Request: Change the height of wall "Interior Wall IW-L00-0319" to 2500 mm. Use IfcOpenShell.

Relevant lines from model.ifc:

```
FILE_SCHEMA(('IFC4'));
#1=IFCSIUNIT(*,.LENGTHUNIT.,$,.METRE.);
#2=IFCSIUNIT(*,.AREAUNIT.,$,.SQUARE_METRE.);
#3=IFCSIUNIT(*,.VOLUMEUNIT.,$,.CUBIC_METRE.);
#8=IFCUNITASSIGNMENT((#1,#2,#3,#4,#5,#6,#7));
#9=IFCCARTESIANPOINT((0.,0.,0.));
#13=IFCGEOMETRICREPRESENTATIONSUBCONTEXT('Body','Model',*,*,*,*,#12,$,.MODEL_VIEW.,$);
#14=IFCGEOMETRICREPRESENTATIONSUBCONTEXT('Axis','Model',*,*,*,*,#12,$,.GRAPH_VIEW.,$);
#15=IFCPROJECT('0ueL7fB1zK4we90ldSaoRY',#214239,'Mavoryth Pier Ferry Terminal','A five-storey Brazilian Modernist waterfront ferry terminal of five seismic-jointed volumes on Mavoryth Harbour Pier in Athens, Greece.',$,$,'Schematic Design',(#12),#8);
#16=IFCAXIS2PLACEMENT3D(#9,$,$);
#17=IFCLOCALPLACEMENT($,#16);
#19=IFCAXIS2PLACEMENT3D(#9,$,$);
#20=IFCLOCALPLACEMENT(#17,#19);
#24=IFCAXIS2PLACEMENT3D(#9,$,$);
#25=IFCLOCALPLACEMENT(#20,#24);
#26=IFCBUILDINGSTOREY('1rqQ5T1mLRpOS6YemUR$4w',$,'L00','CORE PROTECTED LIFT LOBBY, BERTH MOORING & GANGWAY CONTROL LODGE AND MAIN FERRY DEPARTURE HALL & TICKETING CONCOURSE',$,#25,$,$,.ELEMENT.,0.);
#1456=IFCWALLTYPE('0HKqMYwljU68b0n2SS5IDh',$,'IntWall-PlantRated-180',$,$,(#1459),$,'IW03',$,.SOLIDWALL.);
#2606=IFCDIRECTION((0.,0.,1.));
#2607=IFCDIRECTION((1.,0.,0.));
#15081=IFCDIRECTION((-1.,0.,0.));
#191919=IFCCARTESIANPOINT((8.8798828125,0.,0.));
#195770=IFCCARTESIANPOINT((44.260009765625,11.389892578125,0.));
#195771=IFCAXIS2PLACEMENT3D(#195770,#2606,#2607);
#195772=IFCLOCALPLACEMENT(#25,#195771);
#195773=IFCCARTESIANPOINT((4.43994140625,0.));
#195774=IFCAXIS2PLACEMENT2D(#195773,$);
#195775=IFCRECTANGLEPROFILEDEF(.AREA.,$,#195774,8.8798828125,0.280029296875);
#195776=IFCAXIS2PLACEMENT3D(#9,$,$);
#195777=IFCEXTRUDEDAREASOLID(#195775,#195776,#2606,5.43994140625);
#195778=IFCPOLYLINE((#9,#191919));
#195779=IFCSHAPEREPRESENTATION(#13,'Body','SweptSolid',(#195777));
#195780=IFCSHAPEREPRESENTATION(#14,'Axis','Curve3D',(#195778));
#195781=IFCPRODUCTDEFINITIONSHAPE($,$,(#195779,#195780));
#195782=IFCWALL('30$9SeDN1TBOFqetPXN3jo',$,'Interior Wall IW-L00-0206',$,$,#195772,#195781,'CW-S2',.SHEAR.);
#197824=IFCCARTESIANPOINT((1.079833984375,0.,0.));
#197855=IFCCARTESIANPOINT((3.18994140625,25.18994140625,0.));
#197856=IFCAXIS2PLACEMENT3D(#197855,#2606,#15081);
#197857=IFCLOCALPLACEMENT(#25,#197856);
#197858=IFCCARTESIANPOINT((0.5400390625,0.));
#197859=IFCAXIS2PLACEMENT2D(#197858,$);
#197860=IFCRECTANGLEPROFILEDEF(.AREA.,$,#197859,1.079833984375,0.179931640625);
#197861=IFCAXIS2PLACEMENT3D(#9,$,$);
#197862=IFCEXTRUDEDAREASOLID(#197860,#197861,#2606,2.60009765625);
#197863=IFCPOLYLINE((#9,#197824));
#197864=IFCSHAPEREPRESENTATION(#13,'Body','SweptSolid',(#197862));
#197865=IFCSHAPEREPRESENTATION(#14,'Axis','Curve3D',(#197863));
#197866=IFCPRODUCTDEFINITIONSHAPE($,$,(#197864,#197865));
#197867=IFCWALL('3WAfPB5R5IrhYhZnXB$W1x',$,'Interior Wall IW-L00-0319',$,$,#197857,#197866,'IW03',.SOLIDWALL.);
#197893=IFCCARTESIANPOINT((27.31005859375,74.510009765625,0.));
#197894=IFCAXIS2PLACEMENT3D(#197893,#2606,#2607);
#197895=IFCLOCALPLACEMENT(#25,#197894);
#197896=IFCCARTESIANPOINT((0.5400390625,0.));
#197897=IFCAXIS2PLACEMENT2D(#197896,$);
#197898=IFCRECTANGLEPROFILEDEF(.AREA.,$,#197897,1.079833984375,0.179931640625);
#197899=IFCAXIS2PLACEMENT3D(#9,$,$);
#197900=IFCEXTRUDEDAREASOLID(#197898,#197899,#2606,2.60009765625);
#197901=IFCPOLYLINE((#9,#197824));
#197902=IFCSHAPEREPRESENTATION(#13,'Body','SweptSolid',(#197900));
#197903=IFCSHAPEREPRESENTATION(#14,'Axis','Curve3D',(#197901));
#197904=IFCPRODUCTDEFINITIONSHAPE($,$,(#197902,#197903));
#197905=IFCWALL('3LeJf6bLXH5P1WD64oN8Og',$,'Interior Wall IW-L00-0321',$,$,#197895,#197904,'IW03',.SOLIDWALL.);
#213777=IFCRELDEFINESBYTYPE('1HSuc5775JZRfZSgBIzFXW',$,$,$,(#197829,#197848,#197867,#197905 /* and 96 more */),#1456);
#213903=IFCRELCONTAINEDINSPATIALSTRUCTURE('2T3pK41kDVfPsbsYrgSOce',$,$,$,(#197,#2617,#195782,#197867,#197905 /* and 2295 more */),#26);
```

```python
import ifcopenshell
import ifcopenshell.geom
import ifcopenshell.util.representation
import ifcopenshell.util.shape

model = ifcopenshell.open("model.ifc")
settings = ifcopenshell.geom.settings()


def volume(element):
    """Net volume in cubic metres, openings subtracted."""
    shape = ifcopenshell.geom.create_shape(settings, element)
    return ifcopenshell.util.shape.get_volume(shape.geometry)


wall = model.by_guid("3WAfPB5R5IrhYhZnXB$W1x")
before = volume(wall)

body = ifcopenshell.util.representation.get_representation(wall, "Model", "Body")
solid = body.Items[0]
old_height = solid.Depth
solid.Depth = 2.5
after = volume(wall)

print(f"height {old_height:g} -> {solid.Depth:g}, volume {before:.3f} -> {after:.3f} m3")

model.write("model-out.ifc")
```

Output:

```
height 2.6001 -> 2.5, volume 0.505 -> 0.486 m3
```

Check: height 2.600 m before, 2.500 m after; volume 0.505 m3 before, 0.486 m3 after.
